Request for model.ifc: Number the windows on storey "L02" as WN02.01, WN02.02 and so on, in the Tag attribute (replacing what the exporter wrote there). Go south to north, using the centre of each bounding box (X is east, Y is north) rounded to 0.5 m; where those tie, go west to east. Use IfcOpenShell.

First a look at what the model holds.

```python
import ifcopenshell
import ifcopenshell.util.element
import ifcopenshell.util.placement

model = ifcopenshell.open("model.ifc")
print(model.schema)
storey = next(s for s in model.by_type("IfcBuildingStorey") if s.Name == "L02")
windows = [e for e in ifcopenshell.util.element.get_decomposition(storey) if e.is_a("IfcWindow")]
for e in sorted(windows, key=lambda e: e.id()):
    origin = ifcopenshell.util.placement.get_local_placement(e.ObjectPlacement)[:3, 3]
    print(e.id(), e.Tag, e.Name, origin.round(2) + 0.0, sep=" | ")
```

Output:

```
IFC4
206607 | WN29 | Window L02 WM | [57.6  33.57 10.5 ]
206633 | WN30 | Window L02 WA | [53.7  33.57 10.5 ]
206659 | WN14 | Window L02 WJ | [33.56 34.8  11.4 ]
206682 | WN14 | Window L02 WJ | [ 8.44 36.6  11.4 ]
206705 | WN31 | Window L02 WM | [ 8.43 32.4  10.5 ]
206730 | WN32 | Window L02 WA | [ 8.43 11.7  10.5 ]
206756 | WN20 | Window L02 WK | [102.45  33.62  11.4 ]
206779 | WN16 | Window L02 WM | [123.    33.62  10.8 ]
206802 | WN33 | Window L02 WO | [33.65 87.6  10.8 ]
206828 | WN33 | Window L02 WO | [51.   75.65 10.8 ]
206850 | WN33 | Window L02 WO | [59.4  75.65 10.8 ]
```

```python
import ifcopenshell
import ifcopenshell.geom
import ifcopenshell.util.element
import ifcopenshell.util.shape

model = ifcopenshell.open("model.ifc")
settings = ifcopenshell.geom.settings()
settings.set("use-world-coords", True)


def centre(element):
    shape = ifcopenshell.geom.create_shape(settings, element)
    return ifcopenshell.util.shape.get_bbox_centroid(shape.geometry)


storey = next(s for s in model.by_type("IfcBuildingStorey") if s.Name == "L02")
windows = [e for e in ifcopenshell.util.element.get_decomposition(storey) if e.is_a("IfcWindow")]

# Insertion points can sit at a corner or the storey origin, so sort by the geometry (in metres).
centres = {e: centre(e) for e in windows}
windows.sort(key=lambda e: (round(centres[e][1] / 0.5), centres[e][0]))

for i, e in enumerate(windows, start=1):
    number = f"WN02.{i:02d}"
    e.Tag = number
    print(e.id(), number)

model.write("model_rev.ifc")
```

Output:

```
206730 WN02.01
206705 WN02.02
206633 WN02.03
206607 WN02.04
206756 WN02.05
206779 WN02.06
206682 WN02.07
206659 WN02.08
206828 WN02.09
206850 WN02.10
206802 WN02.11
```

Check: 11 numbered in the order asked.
